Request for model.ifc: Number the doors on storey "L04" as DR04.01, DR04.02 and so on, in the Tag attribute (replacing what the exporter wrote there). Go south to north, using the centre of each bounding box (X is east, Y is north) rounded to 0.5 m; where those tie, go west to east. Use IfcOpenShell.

First a look at what the model holds.

```python
import ifcopenshell
import ifcopenshell.util.element
import ifcopenshell.util.placement

model = ifcopenshell.open("model.ifc")
print(model.schema)
storey = next(s for s in model.by_type("IfcBuildingStorey") if s.Name == "L04")
doors = [e for e in ifcopenshell.util.element.get_decomposition(storey) if e.is_a("IfcDoor")]
for e in sorted(doors, key=lambda e: e.id()):
    origin = ifcopenshell.util.placement.get_local_placement(e.ObjectPlacement)[:3, 3]
    print(e.id(), e.Tag, e.Name, origin.round(2) + 0.0, sep=" | ")
```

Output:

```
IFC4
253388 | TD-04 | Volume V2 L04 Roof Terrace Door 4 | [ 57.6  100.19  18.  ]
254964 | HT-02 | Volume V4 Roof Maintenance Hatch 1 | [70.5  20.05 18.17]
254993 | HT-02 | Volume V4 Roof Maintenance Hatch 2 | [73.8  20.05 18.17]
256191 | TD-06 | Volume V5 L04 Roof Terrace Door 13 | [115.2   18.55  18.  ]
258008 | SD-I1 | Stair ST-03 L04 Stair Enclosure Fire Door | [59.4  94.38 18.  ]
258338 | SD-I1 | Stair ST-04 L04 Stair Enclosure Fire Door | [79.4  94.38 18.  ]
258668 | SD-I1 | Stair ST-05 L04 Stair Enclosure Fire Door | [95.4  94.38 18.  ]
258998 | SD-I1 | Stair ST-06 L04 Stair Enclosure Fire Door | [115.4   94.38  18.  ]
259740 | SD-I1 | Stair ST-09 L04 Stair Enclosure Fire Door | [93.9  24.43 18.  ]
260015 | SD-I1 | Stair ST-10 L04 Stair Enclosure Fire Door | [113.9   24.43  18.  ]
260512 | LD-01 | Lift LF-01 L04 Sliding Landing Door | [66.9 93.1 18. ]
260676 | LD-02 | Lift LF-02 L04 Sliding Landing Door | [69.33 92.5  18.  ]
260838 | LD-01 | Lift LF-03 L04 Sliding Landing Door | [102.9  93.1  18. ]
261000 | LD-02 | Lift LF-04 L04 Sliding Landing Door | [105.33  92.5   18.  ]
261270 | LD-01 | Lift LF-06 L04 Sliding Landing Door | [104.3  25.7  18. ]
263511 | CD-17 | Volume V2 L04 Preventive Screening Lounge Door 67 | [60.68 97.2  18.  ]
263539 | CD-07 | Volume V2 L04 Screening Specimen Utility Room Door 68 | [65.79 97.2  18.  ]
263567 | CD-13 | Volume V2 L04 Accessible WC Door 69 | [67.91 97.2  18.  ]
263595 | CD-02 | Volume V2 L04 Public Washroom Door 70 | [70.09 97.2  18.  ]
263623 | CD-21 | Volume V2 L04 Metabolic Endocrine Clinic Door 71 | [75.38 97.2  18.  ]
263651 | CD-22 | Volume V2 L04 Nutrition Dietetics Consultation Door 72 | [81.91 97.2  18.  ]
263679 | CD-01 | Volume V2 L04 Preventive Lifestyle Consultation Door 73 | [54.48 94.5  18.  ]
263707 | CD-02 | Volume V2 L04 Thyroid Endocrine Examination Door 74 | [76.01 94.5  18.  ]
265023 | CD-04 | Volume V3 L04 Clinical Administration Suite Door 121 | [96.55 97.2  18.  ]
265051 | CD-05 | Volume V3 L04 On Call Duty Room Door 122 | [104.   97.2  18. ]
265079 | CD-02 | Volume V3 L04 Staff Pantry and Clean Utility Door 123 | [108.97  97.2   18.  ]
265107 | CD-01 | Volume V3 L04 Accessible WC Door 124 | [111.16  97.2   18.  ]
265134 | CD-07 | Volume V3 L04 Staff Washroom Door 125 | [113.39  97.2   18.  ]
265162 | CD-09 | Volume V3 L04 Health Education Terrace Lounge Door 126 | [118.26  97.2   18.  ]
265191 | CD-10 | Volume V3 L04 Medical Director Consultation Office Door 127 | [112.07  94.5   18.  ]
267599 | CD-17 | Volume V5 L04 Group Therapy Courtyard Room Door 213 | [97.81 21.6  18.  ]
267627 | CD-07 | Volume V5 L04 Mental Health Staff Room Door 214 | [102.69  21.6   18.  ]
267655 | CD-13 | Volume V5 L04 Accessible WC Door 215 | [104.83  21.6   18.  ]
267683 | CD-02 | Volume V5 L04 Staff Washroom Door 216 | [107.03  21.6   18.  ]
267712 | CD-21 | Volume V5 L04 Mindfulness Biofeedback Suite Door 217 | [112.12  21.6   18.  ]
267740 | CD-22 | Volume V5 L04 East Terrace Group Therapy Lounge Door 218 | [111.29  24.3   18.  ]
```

```python
import ifcopenshell
import ifcopenshell.geom
import ifcopenshell.util.element
import ifcopenshell.util.shape

model = ifcopenshell.open("model.ifc")
settings = ifcopenshell.geom.settings()
settings.set("use-world-coords", True)


def centre(element):
    shape = ifcopenshell.geom.create_shape(settings, element)
    return ifcopenshell.util.shape.get_bbox_centroid(shape.geometry)


storey = next(s for s in model.by_type("IfcBuildingStorey") if s.Name == "L04")
doors = [e for e in ifcopenshell.util.element.get_decomposition(storey) if e.is_a("IfcDoor")]

# Insertion points can sit at a corner or the storey origin, so sort by the geometry (in metres).
centres = {e: centre(e) for e in doors}
doors.sort(key=lambda e: (round(centres[e][1] / 0.5), centres[e][0]))

for i, e in enumerate(doors, start=1):
    number = f"DR04.{i:02d}"
    e.Tag = number
    print(e.id(), number)

model.write("model_rev.ifc")
```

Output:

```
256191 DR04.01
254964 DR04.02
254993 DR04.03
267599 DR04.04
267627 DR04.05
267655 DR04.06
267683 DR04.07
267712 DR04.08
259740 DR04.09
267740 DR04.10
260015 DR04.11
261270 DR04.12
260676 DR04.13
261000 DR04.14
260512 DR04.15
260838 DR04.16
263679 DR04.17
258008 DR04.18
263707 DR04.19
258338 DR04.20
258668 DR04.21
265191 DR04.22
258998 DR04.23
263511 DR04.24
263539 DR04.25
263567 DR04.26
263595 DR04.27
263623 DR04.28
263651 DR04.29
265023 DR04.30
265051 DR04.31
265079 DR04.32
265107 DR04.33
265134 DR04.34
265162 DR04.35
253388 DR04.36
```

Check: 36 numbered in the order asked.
